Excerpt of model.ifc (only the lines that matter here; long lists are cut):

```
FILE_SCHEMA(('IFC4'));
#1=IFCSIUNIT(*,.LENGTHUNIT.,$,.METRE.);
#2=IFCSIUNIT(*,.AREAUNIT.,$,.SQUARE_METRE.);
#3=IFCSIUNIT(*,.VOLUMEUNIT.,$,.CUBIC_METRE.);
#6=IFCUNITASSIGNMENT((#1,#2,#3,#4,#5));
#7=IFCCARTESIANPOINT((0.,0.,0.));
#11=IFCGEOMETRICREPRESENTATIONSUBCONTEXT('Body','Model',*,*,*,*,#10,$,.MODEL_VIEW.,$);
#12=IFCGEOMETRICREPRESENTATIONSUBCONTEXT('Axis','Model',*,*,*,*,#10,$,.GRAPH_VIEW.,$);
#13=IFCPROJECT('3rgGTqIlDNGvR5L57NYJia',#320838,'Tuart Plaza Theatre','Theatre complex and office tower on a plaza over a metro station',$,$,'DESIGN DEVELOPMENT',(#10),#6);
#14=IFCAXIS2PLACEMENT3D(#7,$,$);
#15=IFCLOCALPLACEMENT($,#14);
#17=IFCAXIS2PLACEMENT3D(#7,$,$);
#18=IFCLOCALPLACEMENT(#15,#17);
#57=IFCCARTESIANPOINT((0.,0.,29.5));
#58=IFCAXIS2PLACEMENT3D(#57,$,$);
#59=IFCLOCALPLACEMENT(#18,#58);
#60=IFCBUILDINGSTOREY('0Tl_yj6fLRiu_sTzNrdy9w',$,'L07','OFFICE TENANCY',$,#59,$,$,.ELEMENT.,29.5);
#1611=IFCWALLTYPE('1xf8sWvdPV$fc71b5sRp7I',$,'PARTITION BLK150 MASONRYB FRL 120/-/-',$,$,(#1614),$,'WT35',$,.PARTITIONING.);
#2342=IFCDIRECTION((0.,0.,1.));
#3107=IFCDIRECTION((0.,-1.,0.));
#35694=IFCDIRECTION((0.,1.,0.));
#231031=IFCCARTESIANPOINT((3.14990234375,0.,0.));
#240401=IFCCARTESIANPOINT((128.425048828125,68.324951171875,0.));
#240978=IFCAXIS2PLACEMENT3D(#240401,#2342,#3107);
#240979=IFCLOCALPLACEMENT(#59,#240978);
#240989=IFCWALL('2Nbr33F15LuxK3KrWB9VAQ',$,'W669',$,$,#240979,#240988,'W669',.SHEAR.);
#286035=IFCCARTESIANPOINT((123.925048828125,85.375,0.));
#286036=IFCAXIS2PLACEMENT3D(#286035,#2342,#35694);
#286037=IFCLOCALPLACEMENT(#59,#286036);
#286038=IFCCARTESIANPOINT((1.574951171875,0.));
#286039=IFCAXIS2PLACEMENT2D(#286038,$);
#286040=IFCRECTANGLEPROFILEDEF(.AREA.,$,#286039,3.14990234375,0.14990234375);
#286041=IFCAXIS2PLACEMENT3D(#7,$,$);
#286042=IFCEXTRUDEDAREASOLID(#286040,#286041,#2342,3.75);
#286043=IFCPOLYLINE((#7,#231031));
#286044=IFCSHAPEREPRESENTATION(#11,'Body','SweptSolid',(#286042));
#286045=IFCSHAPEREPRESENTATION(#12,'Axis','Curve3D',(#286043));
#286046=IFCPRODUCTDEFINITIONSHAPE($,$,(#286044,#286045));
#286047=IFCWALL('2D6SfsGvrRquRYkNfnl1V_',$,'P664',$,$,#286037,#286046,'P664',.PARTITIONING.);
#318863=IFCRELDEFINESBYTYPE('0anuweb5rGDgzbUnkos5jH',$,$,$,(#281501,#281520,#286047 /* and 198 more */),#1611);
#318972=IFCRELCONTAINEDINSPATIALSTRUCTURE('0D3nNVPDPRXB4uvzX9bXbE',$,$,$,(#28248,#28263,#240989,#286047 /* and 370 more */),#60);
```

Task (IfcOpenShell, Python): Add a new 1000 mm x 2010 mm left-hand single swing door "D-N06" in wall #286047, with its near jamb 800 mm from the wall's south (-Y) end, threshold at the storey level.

```python
import numpy as np
import ifcopenshell
import ifcopenshell.api.feature
import ifcopenshell.api.geometry
import ifcopenshell.api.root
import ifcopenshell.api.spatial
import ifcopenshell.geom
import ifcopenshell.util.element
import ifcopenshell.util.placement
import ifcopenshell.util.representation
import ifcopenshell.util.shape
import ifcopenshell.util.unit

model = ifcopenshell.open("model.ifc")
unit_scale = ifcopenshell.util.unit.calculate_unit_scale(model)
settings = ifcopenshell.geom.settings()


def volume(element):
    """Net volume in cubic metres, openings subtracted."""
    shape = ifcopenshell.geom.create_shape(settings, element)
    return ifcopenshell.util.shape.get_volume(shape.geometry)


wall = model.by_guid("2D6SfsGvrRquRYkNfnl1V_")
storey = ifcopenshell.util.element.get_container(wall, ifc_class="IfcBuildingStorey")
context = ifcopenshell.util.representation.get_context(model, "Model", "Body", "MODEL_VIEW")
before = volume(wall)

width, height, from_end, sill = 1, 2.01, 0.8, 0.0  # metres

# The wall runs along its own X axis, and the end named is its -X end.
wall_shape = ifcopenshell.geom.create_shape(settings, wall)
x, y, z = ifcopenshell.util.shape.get_vertices(wall_shape.geometry).T
start = x.min() + from_end
face, thickness = float(y.min()), float(y.max() - y.min())
wall_matrix = ifcopenshell.util.placement.get_local_placement(wall.ObjectPlacement)
level = ifcopenshell.util.placement.get_local_placement(storey.ObjectPlacement)[2, 3]


def in_wall(x, y):
    """Placement at x, y metres in the wall's axes, at sill height."""
    matrix = wall_matrix.copy()
    matrix[:, 3] = wall_matrix @ np.array([x / unit_scale, y / unit_scale, 0.0, 1.0])
    matrix[2, 3] = level + sill / unit_scale
    return matrix


# Opening: a box that overshoots both wall faces by 50 mm.
opening = ifcopenshell.api.root.create_entity(model, ifc_class="IfcOpeningElement", predefined_type="OPENING")
box = ifcopenshell.api.geometry.add_wall_representation(
    model, context=context, length=width, height=height, thickness=thickness + 0.1
)
ifcopenshell.api.geometry.assign_representation(model, product=opening, representation=box)
ifcopenshell.api.geometry.edit_object_placement(model, product=opening, matrix=in_wall(start, face - 0.05), is_si=False)
ifcopenshell.api.feature.add_feature(model, feature=opening, element=wall)

door = ifcopenshell.api.root.create_entity(model, ifc_class="IfcDoor", name="D-N06", predefined_type="DOOR")
door.OverallWidth, door.OverallHeight = width / unit_scale, height / unit_scale
door.OperationType = "SINGLE_SWING_LEFT"
body = ifcopenshell.api.geometry.add_door_representation(
    model,
    context=context,
    overall_width=door.OverallWidth,
    overall_height=door.OverallHeight,
    operation_type="SINGLE_SWING_LEFT",
    lining_properties={"LiningDepth": thickness / unit_scale, "ThresholdDepth": thickness / unit_scale},
)
ifcopenshell.api.geometry.assign_representation(model, product=door, representation=body)
ifcopenshell.api.spatial.assign_container(model, products=[door], relating_structure=storey)
ifcopenshell.api.feature.add_filling(model, opening=opening, element=door)

# The lining spans the wall, so the door starts at the wall face.
ifcopenshell.api.geometry.edit_object_placement(model, product=door, matrix=in_wall(start, face), is_si=False)

after = volume(wall)

print(f"wall volume {before:.3f} -> {after:.3f} m3")

model.write("model_v2.ifc")
```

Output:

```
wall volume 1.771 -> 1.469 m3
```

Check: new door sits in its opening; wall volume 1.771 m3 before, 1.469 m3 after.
